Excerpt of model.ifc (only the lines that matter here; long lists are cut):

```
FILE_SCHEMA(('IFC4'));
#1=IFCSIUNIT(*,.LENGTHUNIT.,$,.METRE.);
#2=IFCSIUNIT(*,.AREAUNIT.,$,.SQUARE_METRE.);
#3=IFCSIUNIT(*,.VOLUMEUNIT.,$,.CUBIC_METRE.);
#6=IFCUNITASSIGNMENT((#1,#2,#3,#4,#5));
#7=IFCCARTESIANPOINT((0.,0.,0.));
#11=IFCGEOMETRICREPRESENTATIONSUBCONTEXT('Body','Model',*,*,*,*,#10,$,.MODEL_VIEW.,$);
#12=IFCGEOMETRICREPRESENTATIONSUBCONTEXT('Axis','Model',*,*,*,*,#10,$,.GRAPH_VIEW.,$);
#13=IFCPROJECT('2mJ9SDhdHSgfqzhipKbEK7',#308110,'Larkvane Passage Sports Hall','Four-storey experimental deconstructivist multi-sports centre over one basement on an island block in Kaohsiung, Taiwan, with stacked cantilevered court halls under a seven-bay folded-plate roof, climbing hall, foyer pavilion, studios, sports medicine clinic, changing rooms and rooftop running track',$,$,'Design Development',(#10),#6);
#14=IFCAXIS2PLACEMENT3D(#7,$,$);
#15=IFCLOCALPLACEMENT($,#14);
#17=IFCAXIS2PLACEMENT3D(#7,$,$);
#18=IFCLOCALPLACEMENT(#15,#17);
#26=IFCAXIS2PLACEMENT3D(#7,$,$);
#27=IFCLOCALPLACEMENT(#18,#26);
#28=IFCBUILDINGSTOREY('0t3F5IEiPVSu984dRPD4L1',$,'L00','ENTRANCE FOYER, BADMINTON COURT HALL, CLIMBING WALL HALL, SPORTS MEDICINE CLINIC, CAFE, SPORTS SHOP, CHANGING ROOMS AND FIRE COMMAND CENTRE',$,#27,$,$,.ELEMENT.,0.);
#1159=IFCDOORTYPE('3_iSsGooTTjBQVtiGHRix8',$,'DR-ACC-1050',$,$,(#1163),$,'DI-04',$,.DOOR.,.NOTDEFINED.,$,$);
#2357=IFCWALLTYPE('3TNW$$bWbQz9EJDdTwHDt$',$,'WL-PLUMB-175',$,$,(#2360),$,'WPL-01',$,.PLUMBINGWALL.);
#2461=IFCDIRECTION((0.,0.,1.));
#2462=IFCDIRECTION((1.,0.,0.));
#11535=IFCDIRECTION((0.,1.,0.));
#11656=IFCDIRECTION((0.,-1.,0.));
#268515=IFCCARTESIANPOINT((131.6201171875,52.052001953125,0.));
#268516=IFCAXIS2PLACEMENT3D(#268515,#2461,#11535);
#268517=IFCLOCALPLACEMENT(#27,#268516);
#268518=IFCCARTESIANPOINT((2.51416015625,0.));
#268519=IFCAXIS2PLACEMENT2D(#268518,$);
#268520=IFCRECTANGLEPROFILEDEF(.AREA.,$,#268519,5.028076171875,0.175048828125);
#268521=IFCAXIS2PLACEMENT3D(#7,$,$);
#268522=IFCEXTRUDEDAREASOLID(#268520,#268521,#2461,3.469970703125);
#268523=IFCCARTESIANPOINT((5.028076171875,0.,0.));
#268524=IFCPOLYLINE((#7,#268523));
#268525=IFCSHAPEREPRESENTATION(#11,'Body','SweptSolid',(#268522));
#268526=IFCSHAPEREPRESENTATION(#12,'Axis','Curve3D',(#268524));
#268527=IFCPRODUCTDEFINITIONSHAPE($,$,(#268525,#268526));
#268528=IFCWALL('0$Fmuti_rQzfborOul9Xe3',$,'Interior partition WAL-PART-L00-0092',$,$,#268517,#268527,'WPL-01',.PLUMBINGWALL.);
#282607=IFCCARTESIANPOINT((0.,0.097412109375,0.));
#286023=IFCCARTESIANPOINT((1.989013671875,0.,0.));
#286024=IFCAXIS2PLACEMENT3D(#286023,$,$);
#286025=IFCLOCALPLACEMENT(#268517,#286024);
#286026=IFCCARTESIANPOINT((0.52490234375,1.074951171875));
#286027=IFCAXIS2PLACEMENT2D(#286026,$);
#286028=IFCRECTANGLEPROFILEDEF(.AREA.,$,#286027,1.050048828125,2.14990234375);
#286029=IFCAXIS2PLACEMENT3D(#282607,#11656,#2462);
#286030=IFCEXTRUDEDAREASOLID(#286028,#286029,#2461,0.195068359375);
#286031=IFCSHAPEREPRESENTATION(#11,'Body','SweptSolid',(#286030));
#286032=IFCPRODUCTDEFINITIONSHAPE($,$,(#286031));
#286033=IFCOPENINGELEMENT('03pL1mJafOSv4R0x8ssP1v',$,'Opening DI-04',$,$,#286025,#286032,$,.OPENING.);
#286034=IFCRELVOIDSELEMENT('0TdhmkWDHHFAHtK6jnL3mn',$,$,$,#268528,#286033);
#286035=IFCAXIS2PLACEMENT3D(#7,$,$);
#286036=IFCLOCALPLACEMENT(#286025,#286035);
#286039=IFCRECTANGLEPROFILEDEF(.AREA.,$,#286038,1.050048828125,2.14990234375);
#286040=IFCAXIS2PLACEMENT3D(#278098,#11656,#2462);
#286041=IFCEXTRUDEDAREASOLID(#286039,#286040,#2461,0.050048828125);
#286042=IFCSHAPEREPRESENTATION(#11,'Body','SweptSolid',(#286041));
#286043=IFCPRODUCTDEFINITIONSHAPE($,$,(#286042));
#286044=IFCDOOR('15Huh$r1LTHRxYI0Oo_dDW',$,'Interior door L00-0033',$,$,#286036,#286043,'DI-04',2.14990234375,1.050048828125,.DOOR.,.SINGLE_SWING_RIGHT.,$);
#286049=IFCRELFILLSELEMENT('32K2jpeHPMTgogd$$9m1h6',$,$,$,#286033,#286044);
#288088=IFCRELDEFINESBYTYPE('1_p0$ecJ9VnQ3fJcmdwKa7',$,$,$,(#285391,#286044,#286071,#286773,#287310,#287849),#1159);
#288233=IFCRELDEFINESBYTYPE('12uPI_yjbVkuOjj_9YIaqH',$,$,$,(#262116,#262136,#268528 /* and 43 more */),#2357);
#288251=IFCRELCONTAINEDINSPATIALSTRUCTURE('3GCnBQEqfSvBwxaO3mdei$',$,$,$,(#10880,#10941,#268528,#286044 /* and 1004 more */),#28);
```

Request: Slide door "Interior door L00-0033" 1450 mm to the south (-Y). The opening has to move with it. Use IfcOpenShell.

```python
import ifcopenshell
import ifcopenshell.api.geometry
import ifcopenshell.util.placement
import ifcopenshell.util.unit

model = ifcopenshell.open("model.ifc")
unit_scale = ifcopenshell.util.unit.calculate_unit_scale(model)

door = model.by_id(286044)
opening = door.FillsVoids[0].RelatingOpeningElement
wall = opening.VoidsElements[0].RelatingBuildingElement

wall_matrix = ifcopenshell.util.placement.get_local_placement(wall.ObjectPlacement)
shift = wall_matrix[:3, 0] * -1.45 / unit_scale
before = ifcopenshell.util.placement.get_local_placement(door.ObjectPlacement)[:3, 3].copy()

# The door is placed relative to its opening, so it follows when the opening moves.
matrix = ifcopenshell.util.placement.get_local_placement(opening.ObjectPlacement)
matrix[:3, 3] += shift
ifcopenshell.api.geometry.edit_object_placement(
    model, product=opening, matrix=matrix, is_si=False, should_transform_children=True
)

after = ifcopenshell.util.placement.get_local_placement(door.ObjectPlacement)[:3, 3]
print("door moved by", (after - before).round(3) + 0.0)

model.write("model-out.ifc")
```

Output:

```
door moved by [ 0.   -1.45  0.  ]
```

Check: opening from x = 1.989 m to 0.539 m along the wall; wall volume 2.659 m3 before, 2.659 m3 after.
